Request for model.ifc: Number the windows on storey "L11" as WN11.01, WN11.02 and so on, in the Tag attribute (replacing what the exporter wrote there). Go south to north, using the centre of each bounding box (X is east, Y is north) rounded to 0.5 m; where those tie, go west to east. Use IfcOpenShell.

First a look at what the model holds.

```python
import ifcopenshell
import ifcopenshell.util.element
import ifcopenshell.util.placement

model = ifcopenshell.open("model.ifc")
print(model.schema)
storey = next(s for s in model.by_type("IfcBuildingStorey") if s.Name == "L11")
windows = [e for e in ifcopenshell.util.element.get_decomposition(storey) if e.is_a("IfcWindow")]
for e in sorted(windows, key=lambda e: e.id()):
    origin = ifcopenshell.util.placement.get_local_placement(e.ObjectPlacement)[:3, 3]
    print(e.id(), e.Tag, e.Name, origin.round(2) + 0.0, sep=" | ")
```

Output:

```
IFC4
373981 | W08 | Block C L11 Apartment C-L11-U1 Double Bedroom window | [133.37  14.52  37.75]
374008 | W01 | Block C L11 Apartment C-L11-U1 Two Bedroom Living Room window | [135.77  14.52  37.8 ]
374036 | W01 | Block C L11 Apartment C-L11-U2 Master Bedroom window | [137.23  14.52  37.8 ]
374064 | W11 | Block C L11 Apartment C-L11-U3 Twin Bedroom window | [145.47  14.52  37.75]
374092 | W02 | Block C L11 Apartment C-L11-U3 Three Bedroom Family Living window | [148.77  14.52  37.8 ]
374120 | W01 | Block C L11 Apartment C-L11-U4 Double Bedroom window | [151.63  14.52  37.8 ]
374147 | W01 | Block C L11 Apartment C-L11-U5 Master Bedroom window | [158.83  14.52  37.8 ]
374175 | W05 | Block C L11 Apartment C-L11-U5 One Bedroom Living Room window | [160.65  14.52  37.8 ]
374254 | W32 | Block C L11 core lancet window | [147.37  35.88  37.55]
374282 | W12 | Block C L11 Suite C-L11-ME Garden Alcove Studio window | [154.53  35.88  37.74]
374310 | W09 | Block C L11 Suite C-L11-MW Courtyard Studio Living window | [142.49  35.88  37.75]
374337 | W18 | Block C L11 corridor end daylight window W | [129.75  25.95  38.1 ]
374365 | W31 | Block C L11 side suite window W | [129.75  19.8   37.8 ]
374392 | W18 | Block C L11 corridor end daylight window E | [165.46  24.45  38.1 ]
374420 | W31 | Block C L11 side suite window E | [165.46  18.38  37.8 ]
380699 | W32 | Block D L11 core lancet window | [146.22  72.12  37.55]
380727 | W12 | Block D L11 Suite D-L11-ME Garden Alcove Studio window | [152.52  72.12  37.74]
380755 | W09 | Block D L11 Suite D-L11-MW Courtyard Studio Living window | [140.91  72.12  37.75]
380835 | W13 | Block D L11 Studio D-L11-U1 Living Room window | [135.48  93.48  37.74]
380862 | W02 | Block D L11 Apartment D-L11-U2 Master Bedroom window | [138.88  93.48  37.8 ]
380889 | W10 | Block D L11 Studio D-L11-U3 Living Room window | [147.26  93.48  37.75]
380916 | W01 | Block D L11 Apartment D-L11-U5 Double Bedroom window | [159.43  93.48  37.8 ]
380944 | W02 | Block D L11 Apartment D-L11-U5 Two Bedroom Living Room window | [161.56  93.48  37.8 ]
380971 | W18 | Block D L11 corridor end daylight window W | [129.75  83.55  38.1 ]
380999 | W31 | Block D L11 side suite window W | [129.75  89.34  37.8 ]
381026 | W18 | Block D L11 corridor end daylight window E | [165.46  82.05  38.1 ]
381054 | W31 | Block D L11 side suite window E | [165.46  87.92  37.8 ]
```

```python
import ifcopenshell
import ifcopenshell.geom
import ifcopenshell.util.element
import ifcopenshell.util.shape

model = ifcopenshell.open("model.ifc")
settings = ifcopenshell.geom.settings()
settings.set("use-world-coords", True)


def centre(element):
    shape = ifcopenshell.geom.create_shape(settings, element)
    return ifcopenshell.util.shape.get_bbox_centroid(shape.geometry)


storey = next(s for s in model.by_type("IfcBuildingStorey") if s.Name == "L11")
windows = [e for e in ifcopenshell.util.element.get_decomposition(storey) if e.is_a("IfcWindow")]

# Insertion points can sit at a corner or the storey origin, so sort by the geometry (in metres).
centres = {e: centre(e) for e in windows}
windows.sort(key=lambda e: (round(centres[e][1] / 0.5), centres[e][0]))

for i, e in enumerate(windows, start=1):
    number = f"WN11.{i:02d}"
    e.Tag = number
    print(e.id(), number)

model.write("model_edited.ifc")
```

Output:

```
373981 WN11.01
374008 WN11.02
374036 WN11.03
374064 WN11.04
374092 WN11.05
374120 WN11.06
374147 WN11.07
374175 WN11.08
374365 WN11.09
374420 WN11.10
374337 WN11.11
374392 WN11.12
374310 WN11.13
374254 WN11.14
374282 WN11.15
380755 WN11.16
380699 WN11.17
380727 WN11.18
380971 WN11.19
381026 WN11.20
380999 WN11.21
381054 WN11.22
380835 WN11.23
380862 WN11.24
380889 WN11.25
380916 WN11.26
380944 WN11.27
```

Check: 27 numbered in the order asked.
